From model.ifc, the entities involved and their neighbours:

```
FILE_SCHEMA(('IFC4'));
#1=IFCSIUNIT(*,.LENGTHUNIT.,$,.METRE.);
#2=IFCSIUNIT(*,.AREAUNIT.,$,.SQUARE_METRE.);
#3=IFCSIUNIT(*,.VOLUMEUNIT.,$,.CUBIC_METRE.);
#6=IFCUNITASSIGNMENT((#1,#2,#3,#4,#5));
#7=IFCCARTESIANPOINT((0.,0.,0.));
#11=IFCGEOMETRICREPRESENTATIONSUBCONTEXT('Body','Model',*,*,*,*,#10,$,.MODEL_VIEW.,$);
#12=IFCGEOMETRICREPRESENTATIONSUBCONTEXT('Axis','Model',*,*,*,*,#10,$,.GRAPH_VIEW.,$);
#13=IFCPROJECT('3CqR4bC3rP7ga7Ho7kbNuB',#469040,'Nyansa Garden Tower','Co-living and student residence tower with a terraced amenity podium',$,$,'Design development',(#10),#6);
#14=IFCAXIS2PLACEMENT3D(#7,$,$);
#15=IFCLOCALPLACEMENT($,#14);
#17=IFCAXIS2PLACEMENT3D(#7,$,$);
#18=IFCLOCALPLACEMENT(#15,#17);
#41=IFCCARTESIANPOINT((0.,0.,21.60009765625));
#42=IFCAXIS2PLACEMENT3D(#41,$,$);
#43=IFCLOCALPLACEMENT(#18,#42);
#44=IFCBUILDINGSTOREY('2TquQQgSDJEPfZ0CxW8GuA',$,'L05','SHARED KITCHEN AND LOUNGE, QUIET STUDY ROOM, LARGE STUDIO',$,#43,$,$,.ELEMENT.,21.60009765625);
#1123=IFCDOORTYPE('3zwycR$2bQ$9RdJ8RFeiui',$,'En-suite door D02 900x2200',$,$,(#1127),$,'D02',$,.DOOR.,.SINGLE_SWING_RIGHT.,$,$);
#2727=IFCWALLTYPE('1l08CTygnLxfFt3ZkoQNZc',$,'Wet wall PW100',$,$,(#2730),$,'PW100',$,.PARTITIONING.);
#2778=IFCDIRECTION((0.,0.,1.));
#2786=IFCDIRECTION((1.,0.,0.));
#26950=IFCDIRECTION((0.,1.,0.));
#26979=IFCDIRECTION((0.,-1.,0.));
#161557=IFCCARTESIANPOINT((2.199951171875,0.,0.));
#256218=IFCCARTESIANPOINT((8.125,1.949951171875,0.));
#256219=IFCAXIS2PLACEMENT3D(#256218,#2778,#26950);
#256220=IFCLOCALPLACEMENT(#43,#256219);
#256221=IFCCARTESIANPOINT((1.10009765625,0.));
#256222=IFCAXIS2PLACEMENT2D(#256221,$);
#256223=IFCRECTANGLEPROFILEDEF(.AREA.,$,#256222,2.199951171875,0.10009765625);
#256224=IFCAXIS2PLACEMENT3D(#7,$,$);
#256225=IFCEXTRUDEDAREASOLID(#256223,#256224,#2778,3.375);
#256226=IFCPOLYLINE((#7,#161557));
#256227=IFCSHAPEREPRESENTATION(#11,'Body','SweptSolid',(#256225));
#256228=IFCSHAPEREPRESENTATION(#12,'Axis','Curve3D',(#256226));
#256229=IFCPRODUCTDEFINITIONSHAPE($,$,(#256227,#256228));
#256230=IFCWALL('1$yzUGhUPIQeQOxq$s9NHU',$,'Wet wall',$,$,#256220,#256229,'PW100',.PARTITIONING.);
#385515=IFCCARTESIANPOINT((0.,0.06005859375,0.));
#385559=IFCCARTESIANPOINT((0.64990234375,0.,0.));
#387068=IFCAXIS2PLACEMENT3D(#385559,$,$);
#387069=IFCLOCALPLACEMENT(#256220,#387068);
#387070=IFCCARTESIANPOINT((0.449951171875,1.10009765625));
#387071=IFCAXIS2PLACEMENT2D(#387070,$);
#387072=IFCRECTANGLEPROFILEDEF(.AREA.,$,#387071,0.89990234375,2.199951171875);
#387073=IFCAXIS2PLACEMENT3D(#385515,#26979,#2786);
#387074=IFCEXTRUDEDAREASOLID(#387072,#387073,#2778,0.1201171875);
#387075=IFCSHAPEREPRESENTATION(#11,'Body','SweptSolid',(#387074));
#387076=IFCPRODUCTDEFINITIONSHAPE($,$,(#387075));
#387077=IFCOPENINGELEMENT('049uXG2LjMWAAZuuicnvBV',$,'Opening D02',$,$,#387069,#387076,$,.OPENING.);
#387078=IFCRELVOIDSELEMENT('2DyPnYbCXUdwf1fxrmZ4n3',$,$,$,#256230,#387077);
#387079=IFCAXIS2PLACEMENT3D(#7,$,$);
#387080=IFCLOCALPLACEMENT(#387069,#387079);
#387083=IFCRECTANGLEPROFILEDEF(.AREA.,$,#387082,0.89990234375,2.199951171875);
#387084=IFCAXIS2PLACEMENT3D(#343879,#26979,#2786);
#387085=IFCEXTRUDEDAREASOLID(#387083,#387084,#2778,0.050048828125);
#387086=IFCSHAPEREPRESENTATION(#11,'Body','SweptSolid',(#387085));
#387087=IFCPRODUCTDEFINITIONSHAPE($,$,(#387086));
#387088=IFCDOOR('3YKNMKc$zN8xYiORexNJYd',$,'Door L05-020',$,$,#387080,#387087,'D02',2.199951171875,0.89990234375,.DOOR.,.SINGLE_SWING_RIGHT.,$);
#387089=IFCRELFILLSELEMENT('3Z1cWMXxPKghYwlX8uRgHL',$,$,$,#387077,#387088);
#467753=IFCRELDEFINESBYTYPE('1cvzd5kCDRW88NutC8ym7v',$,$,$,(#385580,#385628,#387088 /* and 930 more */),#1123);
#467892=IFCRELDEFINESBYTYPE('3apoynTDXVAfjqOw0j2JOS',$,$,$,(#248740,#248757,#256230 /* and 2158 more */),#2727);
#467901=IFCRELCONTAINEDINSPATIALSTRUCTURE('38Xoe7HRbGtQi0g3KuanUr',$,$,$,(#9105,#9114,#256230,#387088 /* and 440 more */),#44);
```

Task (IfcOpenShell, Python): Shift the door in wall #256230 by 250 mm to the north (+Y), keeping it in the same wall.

```python
import ifcopenshell
import ifcopenshell.api.geometry
import ifcopenshell.util.placement

model = ifcopenshell.open("model.ifc")

door = model.by_guid("3YKNMKc$zN8xYiORexNJYd")
opening = door.FillsVoids[0].RelatingOpeningElement
wall = opening.VoidsElements[0].RelatingBuildingElement

wall_matrix = ifcopenshell.util.placement.get_local_placement(wall.ObjectPlacement)
shift = wall_matrix[:3, 0] * 0.25
before = ifcopenshell.util.placement.get_local_placement(door.ObjectPlacement)[:3, 3].copy()

# The door is placed relative to its opening, so it follows when the opening moves.
matrix = ifcopenshell.util.placement.get_local_placement(opening.ObjectPlacement)
matrix[:3, 3] += shift
ifcopenshell.api.geometry.edit_object_placement(
    model, product=opening, matrix=matrix, is_si=False, should_transform_children=True
)

after = ifcopenshell.util.placement.get_local_placement(door.ObjectPlacement)[:3, 3]
print("door moved by", (after - before).round(3) + 0.0)

model.write("model-out.ifc")
```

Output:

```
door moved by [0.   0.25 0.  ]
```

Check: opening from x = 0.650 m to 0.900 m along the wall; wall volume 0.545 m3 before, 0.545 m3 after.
